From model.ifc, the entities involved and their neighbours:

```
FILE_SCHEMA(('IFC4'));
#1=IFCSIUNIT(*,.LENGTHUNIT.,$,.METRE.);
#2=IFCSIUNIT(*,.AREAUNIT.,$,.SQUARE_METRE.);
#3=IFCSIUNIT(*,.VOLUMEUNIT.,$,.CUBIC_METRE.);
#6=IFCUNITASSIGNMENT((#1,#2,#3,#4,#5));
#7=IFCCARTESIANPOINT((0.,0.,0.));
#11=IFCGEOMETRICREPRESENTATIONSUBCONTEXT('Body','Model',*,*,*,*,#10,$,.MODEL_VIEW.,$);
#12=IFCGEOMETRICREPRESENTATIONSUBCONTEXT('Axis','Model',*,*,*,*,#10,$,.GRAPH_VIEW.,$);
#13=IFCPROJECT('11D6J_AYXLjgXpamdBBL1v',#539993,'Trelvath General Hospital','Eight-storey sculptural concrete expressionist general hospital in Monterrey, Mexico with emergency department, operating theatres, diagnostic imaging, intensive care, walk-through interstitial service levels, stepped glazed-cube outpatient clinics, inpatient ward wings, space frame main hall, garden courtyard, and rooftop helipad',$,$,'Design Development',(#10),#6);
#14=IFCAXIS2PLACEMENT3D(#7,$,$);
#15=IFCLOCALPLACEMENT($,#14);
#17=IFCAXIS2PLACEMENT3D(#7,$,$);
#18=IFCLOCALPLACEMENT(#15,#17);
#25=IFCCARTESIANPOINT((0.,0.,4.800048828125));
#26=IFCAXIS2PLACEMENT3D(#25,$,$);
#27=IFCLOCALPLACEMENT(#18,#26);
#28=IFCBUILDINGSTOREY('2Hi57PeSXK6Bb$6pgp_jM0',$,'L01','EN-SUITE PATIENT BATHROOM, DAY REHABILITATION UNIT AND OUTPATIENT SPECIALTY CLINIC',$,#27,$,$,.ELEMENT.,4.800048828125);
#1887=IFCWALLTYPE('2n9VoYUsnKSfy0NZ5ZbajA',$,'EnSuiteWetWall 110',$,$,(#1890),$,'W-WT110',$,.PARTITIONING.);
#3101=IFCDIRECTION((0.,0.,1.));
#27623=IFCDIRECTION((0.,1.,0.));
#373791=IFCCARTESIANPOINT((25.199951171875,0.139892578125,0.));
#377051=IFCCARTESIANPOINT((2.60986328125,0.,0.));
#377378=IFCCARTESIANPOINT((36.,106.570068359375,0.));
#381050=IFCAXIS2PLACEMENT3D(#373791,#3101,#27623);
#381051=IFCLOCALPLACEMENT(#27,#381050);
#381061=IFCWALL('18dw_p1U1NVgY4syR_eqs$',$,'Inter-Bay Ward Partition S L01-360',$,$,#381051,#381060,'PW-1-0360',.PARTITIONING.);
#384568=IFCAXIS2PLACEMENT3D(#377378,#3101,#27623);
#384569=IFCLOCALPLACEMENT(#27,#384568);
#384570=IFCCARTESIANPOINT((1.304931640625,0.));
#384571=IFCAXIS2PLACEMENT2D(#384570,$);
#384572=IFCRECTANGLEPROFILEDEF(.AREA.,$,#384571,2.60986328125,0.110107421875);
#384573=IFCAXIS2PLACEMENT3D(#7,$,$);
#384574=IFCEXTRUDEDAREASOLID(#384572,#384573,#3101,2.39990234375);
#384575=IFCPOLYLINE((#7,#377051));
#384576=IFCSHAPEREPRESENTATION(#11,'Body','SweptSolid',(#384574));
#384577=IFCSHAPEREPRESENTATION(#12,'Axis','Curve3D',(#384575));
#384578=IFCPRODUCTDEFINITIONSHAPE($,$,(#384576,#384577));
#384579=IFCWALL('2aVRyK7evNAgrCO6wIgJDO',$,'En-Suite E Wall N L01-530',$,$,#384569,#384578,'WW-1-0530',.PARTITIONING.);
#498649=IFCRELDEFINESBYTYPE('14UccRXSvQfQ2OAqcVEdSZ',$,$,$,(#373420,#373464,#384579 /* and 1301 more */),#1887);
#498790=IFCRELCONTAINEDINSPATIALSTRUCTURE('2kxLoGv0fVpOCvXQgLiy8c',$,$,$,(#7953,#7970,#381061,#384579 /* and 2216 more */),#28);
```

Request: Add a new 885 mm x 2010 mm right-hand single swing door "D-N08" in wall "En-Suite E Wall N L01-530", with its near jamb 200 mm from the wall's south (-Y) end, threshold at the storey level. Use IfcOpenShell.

```python
import numpy as np
import ifcopenshell
import ifcopenshell.api.feature
import ifcopenshell.api.geometry
import ifcopenshell.api.root
import ifcopenshell.api.spatial
import ifcopenshell.geom
import ifcopenshell.util.element
import ifcopenshell.util.placement
import ifcopenshell.util.representation
import ifcopenshell.util.shape
import ifcopenshell.util.unit

model = ifcopenshell.open("model.ifc")
unit_scale = ifcopenshell.util.unit.calculate_unit_scale(model)
settings = ifcopenshell.geom.settings()


def volume(element):
    """Net volume in cubic metres, openings subtracted."""
    shape = ifcopenshell.geom.create_shape(settings, element)
    return ifcopenshell.util.shape.get_volume(shape.geometry)


wall = model.by_guid("2aVRyK7evNAgrCO6wIgJDO")
storey = ifcopenshell.util.element.get_container(wall, ifc_class="IfcBuildingStorey")
context = ifcopenshell.util.representation.get_context(model, "Model", "Body", "MODEL_VIEW")
before = volume(wall)

width, height, from_end, sill = 0.885, 2.01, 0.2, 0.0  # metres

# The wall runs along its own X axis, and the end named is its -X end.
wall_shape = ifcopenshell.geom.create_shape(settings, wall)
x, y, z = ifcopenshell.util.shape.get_vertices(wall_shape.geometry).T
start = x.min() + from_end
face, thickness = float(y.min()), float(y.max() - y.min())
wall_matrix = ifcopenshell.util.placement.get_local_placement(wall.ObjectPlacement)
level = ifcopenshell.util.placement.get_local_placement(storey.ObjectPlacement)[2, 3]


def in_wall(x, y):
    """Placement at x, y metres in the wall's axes, at sill height."""
    matrix = wall_matrix.copy()
    matrix[:, 3] = wall_matrix @ np.array([x / unit_scale, y / unit_scale, 0.0, 1.0])
    matrix[2, 3] = level + sill / unit_scale
    return matrix


# Opening: a box that overshoots both wall faces by 50 mm.
opening = ifcopenshell.api.root.create_entity(model, ifc_class="IfcOpeningElement", predefined_type="OPENING")
box = ifcopenshell.api.geometry.add_wall_representation(
    model, context=context, length=width, height=height, thickness=thickness + 0.1
)
ifcopenshell.api.geometry.assign_representation(model, product=opening, representation=box)
ifcopenshell.api.geometry.edit_object_placement(model, product=opening, matrix=in_wall(start, face - 0.05), is_si=False)
ifcopenshell.api.feature.add_feature(model, feature=opening, element=wall)

door = ifcopenshell.api.root.create_entity(model, ifc_class="IfcDoor", name="D-N08", predefined_type="DOOR")
door.OverallWidth, door.OverallHeight = width / unit_scale, height / unit_scale
door.OperationType = "SINGLE_SWING_RIGHT"
body = ifcopenshell.api.geometry.add_door_representation(
    model,
    context=context,
    overall_width=door.OverallWidth,
    overall_height=door.OverallHeight,
    operation_type="SINGLE_SWING_RIGHT",
    lining_properties={"LiningDepth": thickness / unit_scale, "ThresholdDepth": thickness / unit_scale},
)
ifcopenshell.api.geometry.assign_representation(model, product=door, representation=body)
ifcopenshell.api.spatial.assign_container(model, products=[door], relating_structure=storey)
ifcopenshell.api.feature.add_filling(model, opening=opening, element=door)

# The lining spans the wall, so the door starts at the wall face.
ifcopenshell.api.geometry.edit_object_placement(model, product=door, matrix=in_wall(start, face), is_si=False)

after = volume(wall)

print(f"wall volume {before:.3f} -> {after:.3f} m3")

model.write("model_updated.ifc")
```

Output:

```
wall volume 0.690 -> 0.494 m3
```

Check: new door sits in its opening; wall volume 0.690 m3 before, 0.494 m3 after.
